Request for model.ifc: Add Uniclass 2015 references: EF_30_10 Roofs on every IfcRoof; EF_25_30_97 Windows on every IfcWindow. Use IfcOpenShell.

First a look at what the model holds.

```python
import ifcopenshell

model = ifcopenshell.open("model.ifc")
print(model.schema)
print("classifications:", [c.Name for c in model.by_type("IfcClassification")])
for ifc_class in ("IfcDoor", "IfcRoof", "IfcStair", "IfcWall", "IfcWindow"):
    print(ifc_class, len(model.by_type(ifc_class)))
```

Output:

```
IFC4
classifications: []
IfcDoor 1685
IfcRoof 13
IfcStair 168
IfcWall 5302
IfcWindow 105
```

```python
import ifcopenshell
import ifcopenshell.api.classification

model = ifcopenshell.open("model.ifc")

system = ifcopenshell.api.classification.add_classification(model, classification="Uniclass 2015")

codes = {
    "IfcRoof": ("EF_30_10", "Roofs"),
    "IfcWindow": ("EF_25_30_97", "Windows"),
}
for ifc_class, (code, name) in codes.items():
    products = model.by_type(ifc_class)
    ifcopenshell.api.classification.add_reference(
        model, products=products, classification=system, identification=code, name=name
    )
    print(code, len(products))

model.write("model-out.ifc")
```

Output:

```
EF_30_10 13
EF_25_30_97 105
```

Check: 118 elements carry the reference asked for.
